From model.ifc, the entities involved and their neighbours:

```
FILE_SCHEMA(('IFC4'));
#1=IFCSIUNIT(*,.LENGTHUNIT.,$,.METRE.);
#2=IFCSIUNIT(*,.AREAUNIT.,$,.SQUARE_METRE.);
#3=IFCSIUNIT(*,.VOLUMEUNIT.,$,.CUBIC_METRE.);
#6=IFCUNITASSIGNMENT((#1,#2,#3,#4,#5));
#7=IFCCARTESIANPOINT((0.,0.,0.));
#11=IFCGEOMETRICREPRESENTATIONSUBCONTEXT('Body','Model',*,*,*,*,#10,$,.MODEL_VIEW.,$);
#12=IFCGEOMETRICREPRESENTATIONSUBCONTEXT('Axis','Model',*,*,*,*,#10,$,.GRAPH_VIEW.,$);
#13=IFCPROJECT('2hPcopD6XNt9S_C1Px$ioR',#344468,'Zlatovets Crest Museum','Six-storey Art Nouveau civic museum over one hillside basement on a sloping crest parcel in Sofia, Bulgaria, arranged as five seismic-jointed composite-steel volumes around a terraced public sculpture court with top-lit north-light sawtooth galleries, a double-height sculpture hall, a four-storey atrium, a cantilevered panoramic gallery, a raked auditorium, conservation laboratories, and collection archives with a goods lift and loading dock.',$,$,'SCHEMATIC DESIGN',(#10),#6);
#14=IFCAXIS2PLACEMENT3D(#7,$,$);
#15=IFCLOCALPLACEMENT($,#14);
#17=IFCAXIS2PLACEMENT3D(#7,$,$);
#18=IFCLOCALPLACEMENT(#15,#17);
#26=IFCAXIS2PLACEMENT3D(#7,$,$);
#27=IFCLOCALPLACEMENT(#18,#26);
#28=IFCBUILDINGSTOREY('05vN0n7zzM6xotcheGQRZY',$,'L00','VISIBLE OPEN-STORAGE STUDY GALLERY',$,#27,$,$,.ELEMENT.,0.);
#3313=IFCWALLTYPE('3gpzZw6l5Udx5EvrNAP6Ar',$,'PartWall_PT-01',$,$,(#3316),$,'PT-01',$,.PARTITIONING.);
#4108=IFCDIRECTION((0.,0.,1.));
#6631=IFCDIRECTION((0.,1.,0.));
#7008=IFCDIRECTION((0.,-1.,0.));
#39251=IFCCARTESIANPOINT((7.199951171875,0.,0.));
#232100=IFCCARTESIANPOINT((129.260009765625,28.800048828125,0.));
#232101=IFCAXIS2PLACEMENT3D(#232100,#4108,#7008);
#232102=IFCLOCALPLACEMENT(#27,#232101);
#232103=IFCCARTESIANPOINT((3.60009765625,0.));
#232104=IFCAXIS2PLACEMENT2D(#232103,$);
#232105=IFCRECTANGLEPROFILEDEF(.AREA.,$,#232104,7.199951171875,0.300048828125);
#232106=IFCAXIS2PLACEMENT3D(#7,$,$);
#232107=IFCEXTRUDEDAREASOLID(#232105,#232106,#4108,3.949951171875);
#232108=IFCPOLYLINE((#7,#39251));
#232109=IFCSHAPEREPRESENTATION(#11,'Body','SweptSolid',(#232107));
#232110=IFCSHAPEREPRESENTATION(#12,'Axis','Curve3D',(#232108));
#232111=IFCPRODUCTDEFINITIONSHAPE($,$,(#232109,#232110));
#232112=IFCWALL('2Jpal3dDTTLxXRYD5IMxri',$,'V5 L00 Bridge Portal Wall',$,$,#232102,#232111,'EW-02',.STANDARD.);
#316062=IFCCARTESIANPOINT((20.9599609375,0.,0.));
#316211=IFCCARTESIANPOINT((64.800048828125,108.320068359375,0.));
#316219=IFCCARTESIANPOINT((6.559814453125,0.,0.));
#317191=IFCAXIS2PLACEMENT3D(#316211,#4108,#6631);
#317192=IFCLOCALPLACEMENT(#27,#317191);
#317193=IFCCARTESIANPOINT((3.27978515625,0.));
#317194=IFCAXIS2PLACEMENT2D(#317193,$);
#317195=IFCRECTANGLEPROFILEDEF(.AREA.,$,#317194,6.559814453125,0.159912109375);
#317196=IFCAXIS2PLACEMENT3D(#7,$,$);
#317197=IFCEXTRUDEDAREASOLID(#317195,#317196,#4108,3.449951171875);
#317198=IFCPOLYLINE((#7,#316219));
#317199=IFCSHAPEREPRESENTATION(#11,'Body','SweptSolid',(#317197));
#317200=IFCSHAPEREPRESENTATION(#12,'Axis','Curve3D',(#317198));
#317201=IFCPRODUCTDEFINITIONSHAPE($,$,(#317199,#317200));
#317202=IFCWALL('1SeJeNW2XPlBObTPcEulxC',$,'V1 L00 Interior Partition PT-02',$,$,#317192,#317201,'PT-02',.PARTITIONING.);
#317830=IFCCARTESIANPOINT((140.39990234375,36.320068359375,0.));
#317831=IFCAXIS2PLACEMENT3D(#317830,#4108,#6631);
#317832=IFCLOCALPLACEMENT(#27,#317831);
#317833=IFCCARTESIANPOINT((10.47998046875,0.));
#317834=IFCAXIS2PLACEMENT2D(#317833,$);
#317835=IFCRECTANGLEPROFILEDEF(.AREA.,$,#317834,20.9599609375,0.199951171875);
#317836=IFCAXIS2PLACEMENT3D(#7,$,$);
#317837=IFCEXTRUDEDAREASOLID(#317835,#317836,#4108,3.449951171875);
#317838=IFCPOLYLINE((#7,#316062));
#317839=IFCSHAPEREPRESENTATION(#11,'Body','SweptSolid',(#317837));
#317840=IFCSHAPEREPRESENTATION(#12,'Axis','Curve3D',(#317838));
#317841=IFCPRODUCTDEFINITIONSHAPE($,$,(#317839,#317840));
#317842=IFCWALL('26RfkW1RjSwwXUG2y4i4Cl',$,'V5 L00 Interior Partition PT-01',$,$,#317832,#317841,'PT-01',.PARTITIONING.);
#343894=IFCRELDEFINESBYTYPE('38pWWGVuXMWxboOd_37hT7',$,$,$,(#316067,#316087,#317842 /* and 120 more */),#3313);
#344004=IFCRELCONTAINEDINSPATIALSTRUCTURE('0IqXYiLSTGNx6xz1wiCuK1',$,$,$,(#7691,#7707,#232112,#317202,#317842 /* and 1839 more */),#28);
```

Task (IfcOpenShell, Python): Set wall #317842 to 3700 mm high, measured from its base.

```python
import ifcopenshell
import ifcopenshell.geom
import ifcopenshell.util.representation
import ifcopenshell.util.shape

model = ifcopenshell.open("model.ifc")
settings = ifcopenshell.geom.settings()


def volume(element):
    """Net volume in cubic metres, openings subtracted."""
    shape = ifcopenshell.geom.create_shape(settings, element)
    return ifcopenshell.util.shape.get_volume(shape.geometry)


wall = model.by_guid("26RfkW1RjSwwXUG2y4i4Cl")
before = volume(wall)

body = ifcopenshell.util.representation.get_representation(wall, "Model", "Body")
solid = body.Items[0]
old_height = solid.Depth
solid.Depth = 3.7
after = volume(wall)

print(f"height {old_height:g} -> {solid.Depth:g}, volume {before:.3f} -> {after:.3f} m3")

model.write("model_v2.ifc")
```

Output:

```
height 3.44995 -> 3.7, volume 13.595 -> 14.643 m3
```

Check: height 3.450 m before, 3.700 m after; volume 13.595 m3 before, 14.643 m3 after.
